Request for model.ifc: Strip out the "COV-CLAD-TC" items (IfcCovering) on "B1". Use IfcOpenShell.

First a look at what the model holds.

```python
import ifcopenshell
import ifcopenshell.util.element

model = ifcopenshell.open("model.ifc")
print(model.schema)
storey = next(s for s in model.by_type("IfcBuildingStorey") if s.Name == "B1")
coverings = [e for e in ifcopenshell.util.element.get_decomposition(storey) if e.is_a("IfcCovering")]
seen = {}
for e in coverings:
    element_type = ifcopenshell.util.element.get_type(e)
    name = element_type.Name if element_type not in (None, e) else None
    seen[name] = seen.get(name, 0) + 1
for name, count in sorted(seen.items(), key=str):
    print(count, "x", name)
```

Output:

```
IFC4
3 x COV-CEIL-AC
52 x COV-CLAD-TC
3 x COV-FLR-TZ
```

```python
import ifcopenshell
import ifcopenshell.api.root
import ifcopenshell.util.element

model = ifcopenshell.open("model.ifc")

storey = next(s for s in model.by_type("IfcBuildingStorey") if s.Name == "B1")
coverings = [e for e in ifcopenshell.util.element.get_decomposition(storey) if e.is_a("IfcCovering")]
targets = [e for e in coverings if (t := ifcopenshell.util.element.get_type(e)) not in (None, e) and t.Name == "COV-CLAD-TC"]

for e in targets:
    ifcopenshell.api.root.remove_product(model, product=e)
print(len(targets), "removed")

model.write("model_v2.ifc")
```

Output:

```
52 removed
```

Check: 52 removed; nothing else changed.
